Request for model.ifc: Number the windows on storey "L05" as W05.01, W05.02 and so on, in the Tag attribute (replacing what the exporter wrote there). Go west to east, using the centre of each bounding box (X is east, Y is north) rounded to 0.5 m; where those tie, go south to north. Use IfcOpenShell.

First a look at what the model holds.

```python
import ifcopenshell
import ifcopenshell.util.element
import ifcopenshell.util.placement

model = ifcopenshell.open("model.ifc")
print(model.schema)
storey = next(s for s in model.by_type("IfcBuildingStorey") if s.Name == "L05")
windows = [e for e in ifcopenshell.util.element.get_decomposition(storey) if e.is_a("IfcWindow")]
for e in sorted(windows, key=lambda e: e.id()):
    origin = ifcopenshell.util.placement.get_local_placement(e.ObjectPlacement)[:3, 3]
    print(e.id(), e.Tag, e.Name, origin.round(2) + 0.0, sep=" | ")
```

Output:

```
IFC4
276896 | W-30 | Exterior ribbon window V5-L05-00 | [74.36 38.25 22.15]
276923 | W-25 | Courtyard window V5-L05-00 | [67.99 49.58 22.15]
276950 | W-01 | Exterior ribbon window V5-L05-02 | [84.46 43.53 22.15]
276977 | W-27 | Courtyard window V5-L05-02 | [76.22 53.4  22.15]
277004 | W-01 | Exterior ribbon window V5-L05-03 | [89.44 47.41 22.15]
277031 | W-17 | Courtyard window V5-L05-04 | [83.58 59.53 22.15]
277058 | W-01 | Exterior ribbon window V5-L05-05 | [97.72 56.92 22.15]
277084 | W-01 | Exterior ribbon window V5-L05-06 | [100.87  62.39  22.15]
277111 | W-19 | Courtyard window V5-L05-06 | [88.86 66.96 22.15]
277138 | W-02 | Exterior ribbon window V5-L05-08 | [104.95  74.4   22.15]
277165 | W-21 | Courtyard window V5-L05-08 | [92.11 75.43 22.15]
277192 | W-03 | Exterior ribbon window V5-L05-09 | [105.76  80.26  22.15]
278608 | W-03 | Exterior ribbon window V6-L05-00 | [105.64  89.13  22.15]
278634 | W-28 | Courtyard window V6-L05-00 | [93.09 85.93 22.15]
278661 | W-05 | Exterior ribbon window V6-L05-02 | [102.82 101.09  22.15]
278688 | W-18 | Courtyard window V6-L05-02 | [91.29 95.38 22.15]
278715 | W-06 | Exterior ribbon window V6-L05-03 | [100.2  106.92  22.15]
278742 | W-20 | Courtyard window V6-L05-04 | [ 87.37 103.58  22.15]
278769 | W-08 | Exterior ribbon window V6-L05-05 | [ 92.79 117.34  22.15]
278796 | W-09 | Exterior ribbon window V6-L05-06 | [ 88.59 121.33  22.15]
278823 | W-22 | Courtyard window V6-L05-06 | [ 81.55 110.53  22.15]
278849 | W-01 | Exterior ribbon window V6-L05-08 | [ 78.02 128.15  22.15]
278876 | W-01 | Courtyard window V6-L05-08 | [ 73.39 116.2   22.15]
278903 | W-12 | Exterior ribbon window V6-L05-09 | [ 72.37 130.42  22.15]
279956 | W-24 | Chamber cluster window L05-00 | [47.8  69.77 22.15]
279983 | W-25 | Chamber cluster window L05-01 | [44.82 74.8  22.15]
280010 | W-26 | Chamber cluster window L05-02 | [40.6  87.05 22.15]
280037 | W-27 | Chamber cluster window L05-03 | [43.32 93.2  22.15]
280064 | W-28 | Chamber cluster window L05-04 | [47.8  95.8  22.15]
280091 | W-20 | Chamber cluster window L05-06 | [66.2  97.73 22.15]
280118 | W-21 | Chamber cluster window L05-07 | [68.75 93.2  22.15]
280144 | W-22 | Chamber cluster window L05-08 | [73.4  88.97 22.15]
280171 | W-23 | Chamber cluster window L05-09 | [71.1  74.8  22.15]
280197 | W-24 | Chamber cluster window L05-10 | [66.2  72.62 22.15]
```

```python
import ifcopenshell
import ifcopenshell.geom
import ifcopenshell.util.element
import ifcopenshell.util.shape

model = ifcopenshell.open("model.ifc")
settings = ifcopenshell.geom.settings()
settings.set("use-world-coords", True)


def centre(element):
    shape = ifcopenshell.geom.create_shape(settings, element)
    return ifcopenshell.util.shape.get_bbox_centroid(shape.geometry)


storey = next(s for s in model.by_type("IfcBuildingStorey") if s.Name == "L05")
windows = [e for e in ifcopenshell.util.element.get_decomposition(storey) if e.is_a("IfcWindow")]

# Insertion points can sit at a corner or the storey origin, so sort by the geometry (in metres).
centres = {e: centre(e) for e in windows}
windows.sort(key=lambda e: (round(centres[e][0] / 0.5), centres[e][1]))

for i, e in enumerate(windows, start=1):
    number = f"W05.{i:02d}"
    e.Tag = number
    print(e.id(), number)

model.write("model_edited.ifc")
```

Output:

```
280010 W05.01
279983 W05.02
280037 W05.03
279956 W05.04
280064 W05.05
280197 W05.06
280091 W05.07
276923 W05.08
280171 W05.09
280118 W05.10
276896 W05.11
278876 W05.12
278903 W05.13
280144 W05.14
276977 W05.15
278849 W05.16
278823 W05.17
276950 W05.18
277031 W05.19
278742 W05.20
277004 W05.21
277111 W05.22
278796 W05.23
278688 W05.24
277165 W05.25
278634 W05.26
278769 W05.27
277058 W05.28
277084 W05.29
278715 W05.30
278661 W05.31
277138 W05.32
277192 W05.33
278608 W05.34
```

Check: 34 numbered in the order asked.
